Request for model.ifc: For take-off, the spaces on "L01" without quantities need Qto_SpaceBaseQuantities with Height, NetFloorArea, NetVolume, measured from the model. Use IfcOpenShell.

First a look at what the model holds.

```python
import ifcopenshell
import ifcopenshell.util.element
import ifcopenshell.util.unit

model = ifcopenshell.open("model.ifc")
print(model.schema)
for unit_type in ("LENGTHUNIT", "AREAUNIT", "VOLUMEUNIT"):
    print(unit_type, ifcopenshell.util.unit.calculate_unit_scale(model, unit_type))
storey = next(s for s in model.by_type("IfcBuildingStorey") if s.Name == "L01")
spaces = [e for e in ifcopenshell.util.element.get_decomposition(storey) if e.is_a("IfcSpace")]
for e in sorted(spaces, key=lambda e: e.id()):
    print(e.id(), e.is_a(), e.Name, list(ifcopenshell.util.element.get_psets(e, qtos_only=True)), sep=" | ")
```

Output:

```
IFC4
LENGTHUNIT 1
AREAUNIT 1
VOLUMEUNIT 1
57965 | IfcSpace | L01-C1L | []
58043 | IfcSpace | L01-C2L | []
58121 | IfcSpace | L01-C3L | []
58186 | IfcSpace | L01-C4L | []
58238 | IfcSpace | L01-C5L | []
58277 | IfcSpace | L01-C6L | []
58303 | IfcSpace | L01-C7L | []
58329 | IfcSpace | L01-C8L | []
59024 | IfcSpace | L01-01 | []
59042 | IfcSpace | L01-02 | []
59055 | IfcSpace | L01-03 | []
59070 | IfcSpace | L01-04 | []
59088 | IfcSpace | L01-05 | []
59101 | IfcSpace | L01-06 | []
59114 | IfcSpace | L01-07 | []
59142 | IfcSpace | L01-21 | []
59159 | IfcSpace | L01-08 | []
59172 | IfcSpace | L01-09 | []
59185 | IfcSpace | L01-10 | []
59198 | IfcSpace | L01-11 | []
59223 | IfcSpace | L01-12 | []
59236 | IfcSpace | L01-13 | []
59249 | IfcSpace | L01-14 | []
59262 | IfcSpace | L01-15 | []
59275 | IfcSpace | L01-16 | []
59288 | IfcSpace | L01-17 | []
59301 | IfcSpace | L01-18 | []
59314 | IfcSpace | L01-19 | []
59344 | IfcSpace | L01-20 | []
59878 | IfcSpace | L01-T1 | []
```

```python
import ifcopenshell
import ifcopenshell.api.pset
import ifcopenshell.geom
import ifcopenshell.util.element
import ifcopenshell.util.shape
import ifcopenshell.util.unit

model = ifcopenshell.open("model.ifc")
unit_scale = ifcopenshell.util.unit.calculate_unit_scale(model)
area_scale = ifcopenshell.util.unit.calculate_unit_scale(model, "AREAUNIT")
volume_scale = ifcopenshell.util.unit.calculate_unit_scale(model, "VOLUMEUNIT")
settings = ifcopenshell.geom.settings()

storey = next(s for s in model.by_type("IfcBuildingStorey") if s.Name == "L01")
spaces = [e for e in ifcopenshell.util.element.get_decomposition(storey) if e.is_a("IfcSpace")]

for e in sorted(spaces, key=lambda e: e.id()):
    if ifcopenshell.util.element.get_psets(e, qtos_only=True, should_inherit=False):
        continue
    # Geometry comes back in metres, in the element's own axes.
    shape = ifcopenshell.geom.create_shape(settings, e)
    values = {
        "Height": ifcopenshell.util.shape.get_z(shape.geometry) / unit_scale,
        "NetFloorArea": ifcopenshell.util.shape.get_footprint_area(shape.geometry) / area_scale,
        "NetVolume": ifcopenshell.util.shape.get_volume(shape.geometry) / volume_scale,
    }
    qto = ifcopenshell.api.pset.add_qto(model, product=e, name="Qto_SpaceBaseQuantities")
    ifcopenshell.api.pset.edit_qto(model, qto=qto, properties=values)
    print(e.id(), {k: round(v, 3) for k, v in values.items()})

model.write("model_v2.ifc")
```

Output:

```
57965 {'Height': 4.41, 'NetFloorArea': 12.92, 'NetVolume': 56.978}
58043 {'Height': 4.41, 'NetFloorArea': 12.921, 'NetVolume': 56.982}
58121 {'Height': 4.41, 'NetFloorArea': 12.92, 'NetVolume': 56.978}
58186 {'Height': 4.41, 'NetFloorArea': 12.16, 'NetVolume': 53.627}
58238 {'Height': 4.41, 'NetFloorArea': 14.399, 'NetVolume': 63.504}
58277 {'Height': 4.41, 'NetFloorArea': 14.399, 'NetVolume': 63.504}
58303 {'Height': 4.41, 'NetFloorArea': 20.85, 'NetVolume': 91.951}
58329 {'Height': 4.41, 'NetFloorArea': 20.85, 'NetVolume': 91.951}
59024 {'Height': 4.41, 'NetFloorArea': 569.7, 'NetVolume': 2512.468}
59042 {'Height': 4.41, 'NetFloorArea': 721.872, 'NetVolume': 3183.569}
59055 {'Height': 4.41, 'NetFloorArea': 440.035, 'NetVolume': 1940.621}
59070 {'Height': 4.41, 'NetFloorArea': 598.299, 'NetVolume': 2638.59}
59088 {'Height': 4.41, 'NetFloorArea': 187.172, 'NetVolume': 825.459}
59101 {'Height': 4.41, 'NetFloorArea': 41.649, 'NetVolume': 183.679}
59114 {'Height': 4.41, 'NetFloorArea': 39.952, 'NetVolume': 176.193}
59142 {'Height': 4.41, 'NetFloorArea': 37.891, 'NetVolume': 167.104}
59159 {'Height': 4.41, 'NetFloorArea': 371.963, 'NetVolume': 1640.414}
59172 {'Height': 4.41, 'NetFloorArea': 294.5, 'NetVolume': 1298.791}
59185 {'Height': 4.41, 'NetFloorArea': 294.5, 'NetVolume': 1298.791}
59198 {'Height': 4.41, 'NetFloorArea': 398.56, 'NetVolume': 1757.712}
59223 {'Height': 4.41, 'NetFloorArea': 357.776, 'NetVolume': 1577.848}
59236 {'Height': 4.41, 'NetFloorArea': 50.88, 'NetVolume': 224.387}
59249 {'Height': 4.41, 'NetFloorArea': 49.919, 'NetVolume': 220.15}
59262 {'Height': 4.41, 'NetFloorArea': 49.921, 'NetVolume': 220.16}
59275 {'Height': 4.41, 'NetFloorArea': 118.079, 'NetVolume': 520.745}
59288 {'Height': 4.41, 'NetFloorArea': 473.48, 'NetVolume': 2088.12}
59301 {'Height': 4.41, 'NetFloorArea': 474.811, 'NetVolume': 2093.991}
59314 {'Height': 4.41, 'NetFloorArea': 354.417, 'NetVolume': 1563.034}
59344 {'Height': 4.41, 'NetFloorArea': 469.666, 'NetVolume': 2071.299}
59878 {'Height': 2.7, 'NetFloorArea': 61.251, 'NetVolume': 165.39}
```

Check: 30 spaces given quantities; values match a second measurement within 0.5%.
